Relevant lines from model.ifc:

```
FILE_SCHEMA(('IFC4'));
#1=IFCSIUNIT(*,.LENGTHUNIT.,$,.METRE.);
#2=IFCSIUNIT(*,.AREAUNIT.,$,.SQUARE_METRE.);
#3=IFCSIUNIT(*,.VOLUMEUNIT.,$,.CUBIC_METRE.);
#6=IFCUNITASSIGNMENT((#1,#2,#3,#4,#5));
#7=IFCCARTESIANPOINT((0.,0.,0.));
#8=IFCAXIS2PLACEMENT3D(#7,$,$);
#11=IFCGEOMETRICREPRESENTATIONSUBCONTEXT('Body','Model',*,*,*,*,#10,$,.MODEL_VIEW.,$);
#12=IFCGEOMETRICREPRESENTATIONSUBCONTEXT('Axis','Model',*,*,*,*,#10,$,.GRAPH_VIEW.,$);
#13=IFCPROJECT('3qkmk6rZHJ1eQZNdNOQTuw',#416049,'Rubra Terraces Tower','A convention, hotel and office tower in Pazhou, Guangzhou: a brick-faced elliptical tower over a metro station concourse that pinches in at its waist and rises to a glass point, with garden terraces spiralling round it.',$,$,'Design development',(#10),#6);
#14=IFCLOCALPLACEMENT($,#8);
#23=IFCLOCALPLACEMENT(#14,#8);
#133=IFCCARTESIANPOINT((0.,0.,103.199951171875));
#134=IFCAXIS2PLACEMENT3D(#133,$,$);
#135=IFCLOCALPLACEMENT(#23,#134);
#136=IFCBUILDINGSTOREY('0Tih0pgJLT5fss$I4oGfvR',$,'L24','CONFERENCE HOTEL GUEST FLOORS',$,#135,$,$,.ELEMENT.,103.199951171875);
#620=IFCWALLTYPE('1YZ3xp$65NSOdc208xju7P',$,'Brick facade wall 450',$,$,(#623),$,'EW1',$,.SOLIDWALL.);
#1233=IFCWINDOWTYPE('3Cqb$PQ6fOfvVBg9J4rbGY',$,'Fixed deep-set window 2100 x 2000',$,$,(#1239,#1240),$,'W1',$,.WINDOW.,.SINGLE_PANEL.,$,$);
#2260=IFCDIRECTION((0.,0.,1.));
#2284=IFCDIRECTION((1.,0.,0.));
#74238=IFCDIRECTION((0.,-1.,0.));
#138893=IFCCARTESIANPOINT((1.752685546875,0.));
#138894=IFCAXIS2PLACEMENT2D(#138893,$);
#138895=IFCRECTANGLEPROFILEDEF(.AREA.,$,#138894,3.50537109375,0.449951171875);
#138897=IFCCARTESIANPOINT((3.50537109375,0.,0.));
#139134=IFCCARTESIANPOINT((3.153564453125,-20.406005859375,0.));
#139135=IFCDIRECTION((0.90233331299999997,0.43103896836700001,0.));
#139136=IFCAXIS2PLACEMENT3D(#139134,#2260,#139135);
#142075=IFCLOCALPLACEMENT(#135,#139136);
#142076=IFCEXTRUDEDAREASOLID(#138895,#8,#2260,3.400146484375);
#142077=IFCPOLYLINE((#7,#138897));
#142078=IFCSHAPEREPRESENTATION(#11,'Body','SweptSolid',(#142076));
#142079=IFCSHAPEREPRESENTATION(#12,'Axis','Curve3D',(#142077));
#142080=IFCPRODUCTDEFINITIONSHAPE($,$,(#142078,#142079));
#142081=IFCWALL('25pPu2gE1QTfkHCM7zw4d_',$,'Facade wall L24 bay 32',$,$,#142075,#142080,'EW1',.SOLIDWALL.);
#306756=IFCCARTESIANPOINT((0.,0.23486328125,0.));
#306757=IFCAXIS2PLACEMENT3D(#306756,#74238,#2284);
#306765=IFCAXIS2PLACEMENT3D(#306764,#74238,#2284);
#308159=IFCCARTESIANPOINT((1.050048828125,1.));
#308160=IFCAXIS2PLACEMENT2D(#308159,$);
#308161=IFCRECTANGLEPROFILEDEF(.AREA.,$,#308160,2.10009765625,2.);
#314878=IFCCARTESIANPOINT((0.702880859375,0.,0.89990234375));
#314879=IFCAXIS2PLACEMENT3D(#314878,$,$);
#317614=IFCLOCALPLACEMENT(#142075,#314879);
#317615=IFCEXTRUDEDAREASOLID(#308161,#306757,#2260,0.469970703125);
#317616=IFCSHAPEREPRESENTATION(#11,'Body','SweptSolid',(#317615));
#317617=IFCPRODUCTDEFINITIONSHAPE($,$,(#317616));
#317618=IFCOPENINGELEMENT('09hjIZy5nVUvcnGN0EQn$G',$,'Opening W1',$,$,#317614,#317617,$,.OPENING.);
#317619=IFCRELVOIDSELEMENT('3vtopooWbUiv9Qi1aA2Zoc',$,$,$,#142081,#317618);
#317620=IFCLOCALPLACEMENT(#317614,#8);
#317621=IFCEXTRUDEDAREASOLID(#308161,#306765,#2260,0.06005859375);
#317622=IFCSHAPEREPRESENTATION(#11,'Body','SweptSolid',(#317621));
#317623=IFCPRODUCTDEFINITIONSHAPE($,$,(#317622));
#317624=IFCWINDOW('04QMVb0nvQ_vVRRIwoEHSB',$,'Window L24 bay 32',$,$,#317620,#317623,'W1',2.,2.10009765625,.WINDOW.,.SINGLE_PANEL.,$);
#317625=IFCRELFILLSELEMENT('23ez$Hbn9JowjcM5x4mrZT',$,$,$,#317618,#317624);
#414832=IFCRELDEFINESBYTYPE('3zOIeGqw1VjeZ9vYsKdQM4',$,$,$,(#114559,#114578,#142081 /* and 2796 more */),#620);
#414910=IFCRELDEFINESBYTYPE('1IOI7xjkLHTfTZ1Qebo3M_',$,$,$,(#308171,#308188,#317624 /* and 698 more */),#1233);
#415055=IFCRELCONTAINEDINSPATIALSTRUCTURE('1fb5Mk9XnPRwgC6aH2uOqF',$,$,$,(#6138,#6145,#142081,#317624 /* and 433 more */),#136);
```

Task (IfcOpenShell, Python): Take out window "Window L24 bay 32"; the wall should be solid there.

```python
import ifcopenshell
import ifcopenshell.api.feature
import ifcopenshell.api.root
import ifcopenshell.geom
import ifcopenshell.util.shape

model = ifcopenshell.open("model.ifc")
settings = ifcopenshell.geom.settings()


def volume(element):
    """Net volume in cubic metres, openings subtracted."""
    shape = ifcopenshell.geom.create_shape(settings, element)
    return ifcopenshell.util.shape.get_volume(shape.geometry)


window = model.by_guid("04QMVb0nvQ_vVRRIwoEHSB")
opening = window.FillsVoids[0].RelatingOpeningElement
wall = opening.VoidsElements[0].RelatingBuildingElement
before = volume(wall)

ifcopenshell.api.root.remove_product(model, product=window)
ifcopenshell.api.feature.remove_feature(model, feature=opening)

after = volume(wall)

print(f"wall volume {before:.3f} -> {after:.3f} m3")

model.write("model-out.ifc")
```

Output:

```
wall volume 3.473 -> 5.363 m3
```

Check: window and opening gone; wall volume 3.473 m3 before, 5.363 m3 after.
